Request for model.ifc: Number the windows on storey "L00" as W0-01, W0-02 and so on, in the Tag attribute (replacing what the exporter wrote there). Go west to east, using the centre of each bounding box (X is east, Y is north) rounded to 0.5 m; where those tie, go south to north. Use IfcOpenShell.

First a look at what the model holds.

```python
import ifcopenshell
import ifcopenshell.util.element
import ifcopenshell.util.placement

model = ifcopenshell.open("model.ifc")
print(model.schema)
storey = next(s for s in model.by_type("IfcBuildingStorey") if s.Name == "L00")
windows = [e for e in ifcopenshell.util.element.get_decomposition(storey) if e.is_a("IfcWindow")]
for e in sorted(windows, key=lambda e: e.id()):
    origin = ifcopenshell.util.placement.get_local_placement(e.ObjectPlacement)[:3, 3]
    print(e.id(), e.Tag, e.Name, origin.round(2) + 0.0, sep=" | ")
```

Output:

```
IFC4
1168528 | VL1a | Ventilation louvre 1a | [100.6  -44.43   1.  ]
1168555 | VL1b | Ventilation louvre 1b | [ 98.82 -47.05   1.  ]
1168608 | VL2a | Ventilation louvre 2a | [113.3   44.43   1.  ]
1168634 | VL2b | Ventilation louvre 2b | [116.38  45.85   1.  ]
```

```python
import ifcopenshell
import ifcopenshell.geom
import ifcopenshell.util.element
import ifcopenshell.util.shape

model = ifcopenshell.open("model.ifc")
settings = ifcopenshell.geom.settings()
settings.set("use-world-coords", True)


def centre(element):
    shape = ifcopenshell.geom.create_shape(settings, element)
    return ifcopenshell.util.shape.get_bbox_centroid(shape.geometry)


storey = next(s for s in model.by_type("IfcBuildingStorey") if s.Name == "L00")
windows = [e for e in ifcopenshell.util.element.get_decomposition(storey) if e.is_a("IfcWindow")]

# Insertion points can sit at a corner or the storey origin, so sort by the geometry (in metres).
centres = {e: centre(e) for e in windows}
windows.sort(key=lambda e: (round(centres[e][0] / 0.5), centres[e][1]))

for i, e in enumerate(windows, start=1):
    number = f"W0-{i:02d}"
    e.Tag = number
    print(e.id(), number)

model.write("model_edited.ifc")
```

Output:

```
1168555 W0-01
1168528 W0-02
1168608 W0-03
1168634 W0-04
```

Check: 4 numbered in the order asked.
